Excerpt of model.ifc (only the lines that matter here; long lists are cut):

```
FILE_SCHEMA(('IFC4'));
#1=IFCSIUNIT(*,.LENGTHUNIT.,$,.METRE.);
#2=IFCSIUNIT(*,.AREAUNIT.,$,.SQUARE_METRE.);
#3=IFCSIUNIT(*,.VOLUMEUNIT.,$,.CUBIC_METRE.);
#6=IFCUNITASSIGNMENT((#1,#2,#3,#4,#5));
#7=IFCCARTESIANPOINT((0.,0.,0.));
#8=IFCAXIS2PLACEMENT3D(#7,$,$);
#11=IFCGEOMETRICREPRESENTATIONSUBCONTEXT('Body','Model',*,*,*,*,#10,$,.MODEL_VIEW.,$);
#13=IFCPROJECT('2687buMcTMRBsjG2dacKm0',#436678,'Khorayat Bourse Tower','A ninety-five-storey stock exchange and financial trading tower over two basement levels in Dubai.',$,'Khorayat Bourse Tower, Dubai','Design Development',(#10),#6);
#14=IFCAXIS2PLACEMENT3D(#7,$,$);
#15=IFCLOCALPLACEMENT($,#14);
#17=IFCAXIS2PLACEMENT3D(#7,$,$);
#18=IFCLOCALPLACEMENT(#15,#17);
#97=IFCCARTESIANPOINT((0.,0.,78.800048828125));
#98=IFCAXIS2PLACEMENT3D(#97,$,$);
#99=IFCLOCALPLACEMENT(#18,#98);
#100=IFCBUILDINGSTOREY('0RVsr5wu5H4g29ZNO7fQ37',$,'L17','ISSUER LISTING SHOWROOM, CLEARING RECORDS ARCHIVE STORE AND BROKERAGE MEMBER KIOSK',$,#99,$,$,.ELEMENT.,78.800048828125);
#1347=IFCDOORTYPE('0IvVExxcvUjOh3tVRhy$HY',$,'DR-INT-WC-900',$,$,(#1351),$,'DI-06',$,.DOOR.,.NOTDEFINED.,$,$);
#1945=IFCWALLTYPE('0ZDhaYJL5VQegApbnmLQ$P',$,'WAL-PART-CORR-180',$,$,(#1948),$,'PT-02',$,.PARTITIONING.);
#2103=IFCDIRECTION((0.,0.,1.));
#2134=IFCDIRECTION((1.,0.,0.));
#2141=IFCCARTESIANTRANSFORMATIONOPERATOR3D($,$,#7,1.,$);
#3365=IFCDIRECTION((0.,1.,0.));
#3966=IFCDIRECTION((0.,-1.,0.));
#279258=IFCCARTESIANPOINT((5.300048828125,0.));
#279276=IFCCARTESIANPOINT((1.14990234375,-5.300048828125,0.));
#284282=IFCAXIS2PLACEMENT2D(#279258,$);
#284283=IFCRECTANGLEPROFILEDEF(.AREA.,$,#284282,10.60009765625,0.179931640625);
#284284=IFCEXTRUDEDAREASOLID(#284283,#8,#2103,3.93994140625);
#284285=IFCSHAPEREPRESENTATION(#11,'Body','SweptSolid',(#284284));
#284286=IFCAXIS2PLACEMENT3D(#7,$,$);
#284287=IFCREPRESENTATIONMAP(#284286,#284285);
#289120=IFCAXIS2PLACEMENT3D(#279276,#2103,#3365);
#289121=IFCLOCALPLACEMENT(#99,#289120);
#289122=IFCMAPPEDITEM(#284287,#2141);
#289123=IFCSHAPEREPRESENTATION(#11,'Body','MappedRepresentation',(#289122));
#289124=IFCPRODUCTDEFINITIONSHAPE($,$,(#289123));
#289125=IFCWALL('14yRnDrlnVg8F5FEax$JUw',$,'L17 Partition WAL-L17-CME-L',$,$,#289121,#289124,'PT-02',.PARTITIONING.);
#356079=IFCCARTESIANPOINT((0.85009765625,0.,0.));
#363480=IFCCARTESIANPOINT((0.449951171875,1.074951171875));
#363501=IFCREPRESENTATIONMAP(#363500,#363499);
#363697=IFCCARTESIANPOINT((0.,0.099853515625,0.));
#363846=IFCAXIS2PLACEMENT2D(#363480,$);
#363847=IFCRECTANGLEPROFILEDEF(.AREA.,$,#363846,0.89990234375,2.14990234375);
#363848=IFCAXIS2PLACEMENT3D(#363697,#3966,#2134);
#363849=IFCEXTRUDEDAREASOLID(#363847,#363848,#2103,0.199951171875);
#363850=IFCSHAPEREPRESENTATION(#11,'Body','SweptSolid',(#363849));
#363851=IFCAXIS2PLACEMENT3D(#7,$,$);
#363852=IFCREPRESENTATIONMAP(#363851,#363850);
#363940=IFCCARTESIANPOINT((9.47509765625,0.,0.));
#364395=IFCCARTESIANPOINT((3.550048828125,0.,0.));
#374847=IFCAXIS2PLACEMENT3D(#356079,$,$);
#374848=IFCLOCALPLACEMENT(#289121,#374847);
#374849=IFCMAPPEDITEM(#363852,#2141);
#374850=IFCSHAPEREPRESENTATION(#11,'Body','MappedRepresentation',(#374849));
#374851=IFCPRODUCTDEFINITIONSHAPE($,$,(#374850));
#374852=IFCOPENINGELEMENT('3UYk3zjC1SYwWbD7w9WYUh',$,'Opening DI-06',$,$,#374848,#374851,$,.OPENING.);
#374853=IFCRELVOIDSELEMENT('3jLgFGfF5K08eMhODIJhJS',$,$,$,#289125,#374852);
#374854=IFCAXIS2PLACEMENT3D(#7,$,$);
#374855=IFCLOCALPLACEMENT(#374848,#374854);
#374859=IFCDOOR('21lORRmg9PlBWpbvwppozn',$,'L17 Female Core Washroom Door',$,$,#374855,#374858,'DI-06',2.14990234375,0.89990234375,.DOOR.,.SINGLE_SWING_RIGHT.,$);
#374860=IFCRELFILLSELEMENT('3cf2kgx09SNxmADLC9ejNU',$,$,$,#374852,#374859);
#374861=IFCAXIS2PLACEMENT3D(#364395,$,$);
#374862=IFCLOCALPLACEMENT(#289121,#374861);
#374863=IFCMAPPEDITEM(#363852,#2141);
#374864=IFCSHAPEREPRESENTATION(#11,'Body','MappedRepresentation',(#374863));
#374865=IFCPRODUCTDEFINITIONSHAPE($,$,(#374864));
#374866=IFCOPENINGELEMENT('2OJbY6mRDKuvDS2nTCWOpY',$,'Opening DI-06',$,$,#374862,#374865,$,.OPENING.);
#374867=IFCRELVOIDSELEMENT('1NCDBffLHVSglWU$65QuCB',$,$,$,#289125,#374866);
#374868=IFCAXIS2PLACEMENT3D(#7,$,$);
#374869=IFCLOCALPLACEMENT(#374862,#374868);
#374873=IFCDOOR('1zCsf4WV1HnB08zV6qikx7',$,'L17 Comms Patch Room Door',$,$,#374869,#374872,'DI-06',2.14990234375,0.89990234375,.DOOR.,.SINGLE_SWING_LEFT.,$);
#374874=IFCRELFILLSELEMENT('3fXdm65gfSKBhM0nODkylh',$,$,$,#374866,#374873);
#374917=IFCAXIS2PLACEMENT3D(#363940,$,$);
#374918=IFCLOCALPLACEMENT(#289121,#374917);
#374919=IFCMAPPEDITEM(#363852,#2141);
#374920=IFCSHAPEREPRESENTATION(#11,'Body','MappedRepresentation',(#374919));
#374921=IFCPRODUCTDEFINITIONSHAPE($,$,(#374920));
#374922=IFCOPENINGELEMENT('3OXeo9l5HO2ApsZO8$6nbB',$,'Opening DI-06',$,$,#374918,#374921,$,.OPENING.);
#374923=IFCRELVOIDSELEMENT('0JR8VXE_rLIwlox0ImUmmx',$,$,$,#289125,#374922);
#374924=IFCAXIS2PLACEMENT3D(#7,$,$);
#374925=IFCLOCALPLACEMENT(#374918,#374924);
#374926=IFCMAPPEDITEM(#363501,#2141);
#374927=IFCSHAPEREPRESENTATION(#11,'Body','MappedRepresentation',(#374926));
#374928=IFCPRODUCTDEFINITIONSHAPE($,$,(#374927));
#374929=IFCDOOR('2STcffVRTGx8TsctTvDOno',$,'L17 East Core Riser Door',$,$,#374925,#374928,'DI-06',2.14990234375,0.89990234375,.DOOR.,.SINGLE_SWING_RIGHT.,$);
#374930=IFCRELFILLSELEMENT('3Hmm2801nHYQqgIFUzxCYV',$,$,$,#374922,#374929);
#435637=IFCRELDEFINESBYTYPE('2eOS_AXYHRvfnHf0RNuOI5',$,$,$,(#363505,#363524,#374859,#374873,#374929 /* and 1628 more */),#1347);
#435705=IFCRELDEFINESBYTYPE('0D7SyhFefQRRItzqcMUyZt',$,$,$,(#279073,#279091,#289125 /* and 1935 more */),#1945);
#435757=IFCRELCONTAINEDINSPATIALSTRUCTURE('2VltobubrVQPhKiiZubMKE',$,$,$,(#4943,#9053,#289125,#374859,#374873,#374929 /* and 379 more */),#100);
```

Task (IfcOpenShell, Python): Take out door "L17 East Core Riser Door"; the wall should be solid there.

```python
import ifcopenshell
import ifcopenshell.api.feature
import ifcopenshell.api.root
import ifcopenshell.geom
import ifcopenshell.util.shape

model = ifcopenshell.open("model.ifc")
settings = ifcopenshell.geom.settings()


def volume(element):
    """Net volume in cubic metres, openings subtracted."""
    shape = ifcopenshell.geom.create_shape(settings, element)
    return ifcopenshell.util.shape.get_volume(shape.geometry)


door = model.by_id(374929)
opening = door.FillsVoids[0].RelatingOpeningElement
wall = opening.VoidsElements[0].RelatingBuildingElement
before = volume(wall)

ifcopenshell.api.root.remove_product(model, product=door)
ifcopenshell.api.feature.remove_feature(model, feature=opening)

after = volume(wall)

print(f"wall volume {before:.3f} -> {after:.3f} m3")

model.write("model_v2.ifc")
```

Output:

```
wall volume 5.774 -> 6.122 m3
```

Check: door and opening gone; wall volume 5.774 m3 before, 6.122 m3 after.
